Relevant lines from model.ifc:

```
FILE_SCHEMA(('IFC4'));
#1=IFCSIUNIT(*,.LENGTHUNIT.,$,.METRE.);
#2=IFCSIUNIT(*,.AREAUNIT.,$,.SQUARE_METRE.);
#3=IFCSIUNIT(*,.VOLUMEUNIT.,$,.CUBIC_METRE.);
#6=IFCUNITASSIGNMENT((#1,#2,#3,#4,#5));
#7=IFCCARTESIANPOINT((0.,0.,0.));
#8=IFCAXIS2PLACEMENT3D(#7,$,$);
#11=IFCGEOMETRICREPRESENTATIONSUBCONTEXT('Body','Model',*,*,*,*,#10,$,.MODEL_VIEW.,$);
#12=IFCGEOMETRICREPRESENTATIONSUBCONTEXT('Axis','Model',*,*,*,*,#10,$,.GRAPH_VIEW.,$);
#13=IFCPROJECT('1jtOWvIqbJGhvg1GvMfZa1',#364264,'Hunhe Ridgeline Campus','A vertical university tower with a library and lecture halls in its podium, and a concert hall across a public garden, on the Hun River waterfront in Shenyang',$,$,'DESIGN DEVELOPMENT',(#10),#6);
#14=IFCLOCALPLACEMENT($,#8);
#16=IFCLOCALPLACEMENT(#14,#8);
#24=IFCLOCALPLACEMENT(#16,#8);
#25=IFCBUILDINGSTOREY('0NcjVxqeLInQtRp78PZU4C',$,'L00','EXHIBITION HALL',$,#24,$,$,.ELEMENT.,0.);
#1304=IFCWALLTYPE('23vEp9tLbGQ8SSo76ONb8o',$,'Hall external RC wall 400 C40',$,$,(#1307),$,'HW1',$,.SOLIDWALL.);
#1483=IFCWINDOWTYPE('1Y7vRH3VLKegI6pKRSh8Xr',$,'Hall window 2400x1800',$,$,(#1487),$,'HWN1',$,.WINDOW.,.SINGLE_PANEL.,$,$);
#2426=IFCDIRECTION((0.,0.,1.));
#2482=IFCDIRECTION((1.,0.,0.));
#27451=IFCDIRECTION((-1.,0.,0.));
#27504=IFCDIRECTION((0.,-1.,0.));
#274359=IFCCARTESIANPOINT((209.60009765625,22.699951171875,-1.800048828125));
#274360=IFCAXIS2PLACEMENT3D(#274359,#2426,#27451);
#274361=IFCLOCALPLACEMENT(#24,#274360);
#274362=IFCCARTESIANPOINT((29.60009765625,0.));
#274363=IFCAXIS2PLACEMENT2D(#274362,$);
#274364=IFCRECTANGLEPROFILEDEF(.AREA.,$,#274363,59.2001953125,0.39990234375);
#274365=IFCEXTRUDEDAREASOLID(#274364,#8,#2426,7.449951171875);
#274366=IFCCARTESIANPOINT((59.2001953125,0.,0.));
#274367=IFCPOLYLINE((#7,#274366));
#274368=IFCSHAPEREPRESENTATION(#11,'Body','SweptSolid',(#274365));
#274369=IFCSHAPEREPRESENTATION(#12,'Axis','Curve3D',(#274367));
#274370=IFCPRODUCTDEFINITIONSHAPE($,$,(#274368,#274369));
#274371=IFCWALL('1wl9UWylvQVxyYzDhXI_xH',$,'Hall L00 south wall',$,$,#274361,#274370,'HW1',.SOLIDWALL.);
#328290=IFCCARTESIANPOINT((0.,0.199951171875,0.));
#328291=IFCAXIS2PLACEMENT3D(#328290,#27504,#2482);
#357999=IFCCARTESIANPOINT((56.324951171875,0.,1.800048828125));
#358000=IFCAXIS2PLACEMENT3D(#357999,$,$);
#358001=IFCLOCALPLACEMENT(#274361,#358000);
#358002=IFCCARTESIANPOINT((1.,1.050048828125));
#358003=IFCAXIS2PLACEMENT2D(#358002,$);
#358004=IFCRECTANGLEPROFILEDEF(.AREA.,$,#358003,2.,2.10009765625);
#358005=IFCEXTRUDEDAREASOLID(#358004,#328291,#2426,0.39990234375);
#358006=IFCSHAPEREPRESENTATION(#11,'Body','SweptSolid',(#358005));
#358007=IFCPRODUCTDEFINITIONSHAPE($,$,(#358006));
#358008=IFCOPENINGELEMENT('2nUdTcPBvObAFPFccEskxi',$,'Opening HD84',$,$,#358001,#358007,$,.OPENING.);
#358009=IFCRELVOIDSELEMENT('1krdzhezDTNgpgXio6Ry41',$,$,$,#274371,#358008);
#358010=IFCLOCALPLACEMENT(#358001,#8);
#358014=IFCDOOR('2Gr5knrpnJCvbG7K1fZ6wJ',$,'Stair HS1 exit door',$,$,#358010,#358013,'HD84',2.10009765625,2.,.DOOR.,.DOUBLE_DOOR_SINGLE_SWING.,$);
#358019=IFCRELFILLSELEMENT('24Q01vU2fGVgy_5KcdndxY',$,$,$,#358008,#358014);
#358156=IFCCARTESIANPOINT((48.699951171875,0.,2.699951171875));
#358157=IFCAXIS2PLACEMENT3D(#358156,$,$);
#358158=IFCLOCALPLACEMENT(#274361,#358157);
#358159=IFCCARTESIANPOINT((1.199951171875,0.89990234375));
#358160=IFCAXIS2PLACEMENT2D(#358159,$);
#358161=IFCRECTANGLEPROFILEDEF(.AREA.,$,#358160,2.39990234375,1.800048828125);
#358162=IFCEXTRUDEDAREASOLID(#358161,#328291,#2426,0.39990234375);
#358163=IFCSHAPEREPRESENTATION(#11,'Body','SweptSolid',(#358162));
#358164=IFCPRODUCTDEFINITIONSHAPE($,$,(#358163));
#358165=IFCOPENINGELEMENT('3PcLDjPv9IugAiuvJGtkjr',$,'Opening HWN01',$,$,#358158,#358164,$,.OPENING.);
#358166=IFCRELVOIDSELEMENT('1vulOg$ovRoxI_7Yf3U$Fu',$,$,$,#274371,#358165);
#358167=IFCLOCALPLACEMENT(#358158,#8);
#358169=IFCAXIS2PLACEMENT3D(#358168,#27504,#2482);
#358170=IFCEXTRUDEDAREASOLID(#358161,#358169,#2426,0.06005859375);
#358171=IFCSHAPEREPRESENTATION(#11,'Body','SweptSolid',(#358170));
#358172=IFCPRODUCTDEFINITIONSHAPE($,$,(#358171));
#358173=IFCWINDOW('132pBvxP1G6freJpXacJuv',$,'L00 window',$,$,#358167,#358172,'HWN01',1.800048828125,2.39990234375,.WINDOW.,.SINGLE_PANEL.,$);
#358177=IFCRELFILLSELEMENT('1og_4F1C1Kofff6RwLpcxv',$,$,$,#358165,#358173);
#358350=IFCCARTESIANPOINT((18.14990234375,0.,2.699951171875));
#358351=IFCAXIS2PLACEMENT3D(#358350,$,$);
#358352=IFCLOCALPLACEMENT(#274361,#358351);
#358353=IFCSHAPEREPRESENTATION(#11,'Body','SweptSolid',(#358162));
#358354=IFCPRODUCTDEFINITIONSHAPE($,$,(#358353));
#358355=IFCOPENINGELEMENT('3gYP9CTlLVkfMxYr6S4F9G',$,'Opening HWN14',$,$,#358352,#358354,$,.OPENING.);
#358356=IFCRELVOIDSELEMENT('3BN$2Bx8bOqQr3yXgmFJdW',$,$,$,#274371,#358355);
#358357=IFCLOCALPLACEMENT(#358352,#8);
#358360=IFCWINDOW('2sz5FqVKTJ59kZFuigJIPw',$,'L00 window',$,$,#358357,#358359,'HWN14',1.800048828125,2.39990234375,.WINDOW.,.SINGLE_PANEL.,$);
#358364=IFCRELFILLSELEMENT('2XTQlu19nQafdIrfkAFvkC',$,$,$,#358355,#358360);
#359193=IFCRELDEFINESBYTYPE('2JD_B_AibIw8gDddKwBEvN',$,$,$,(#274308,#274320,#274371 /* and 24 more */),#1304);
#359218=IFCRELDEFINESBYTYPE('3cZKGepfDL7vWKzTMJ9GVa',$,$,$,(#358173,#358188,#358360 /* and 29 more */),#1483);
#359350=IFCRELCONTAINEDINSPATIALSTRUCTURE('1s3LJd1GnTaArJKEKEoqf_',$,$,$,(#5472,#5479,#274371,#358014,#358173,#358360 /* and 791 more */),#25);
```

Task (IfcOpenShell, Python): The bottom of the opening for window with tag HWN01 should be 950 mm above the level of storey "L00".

```python
import numpy as np
import ifcopenshell
import ifcopenshell.api.geometry
import ifcopenshell.geom
import ifcopenshell.util.element
import ifcopenshell.util.placement
import ifcopenshell.util.shape
import ifcopenshell.util.unit

model = ifcopenshell.open("model.ifc")
unit_scale = ifcopenshell.util.unit.calculate_unit_scale(model)

window = model.by_guid("132pBvxP1G6freJpXacJuv")
opening = window.FillsVoids[0].RelatingOpeningElement
storey = ifcopenshell.util.element.get_container(window, ifc_class="IfcBuildingStorey")
level = ifcopenshell.util.placement.get_local_placement(storey.ObjectPlacement)[2, 3]

# The opening's origin need not be at the sill, so measure its lowest point.
shape = ifcopenshell.geom.create_shape(ifcopenshell.geom.settings(), opening)
bottom = ifcopenshell.util.shape.get_shape_bottom_elevation(shape, shape.geometry) / unit_scale
dz = level + 0.95 / unit_scale - bottom

shift = np.array([0.0, 0.0, dz])
# The window is placed relative to its opening, so it follows when the opening moves.
matrix = ifcopenshell.util.placement.get_local_placement(opening.ObjectPlacement)
matrix[:3, 3] += shift
ifcopenshell.api.geometry.edit_object_placement(
    model, product=opening, matrix=matrix, is_si=False, should_transform_children=True
)

print(f"moved by {dz * unit_scale:+.3f} m")

model.write("model_rev.ifc")
```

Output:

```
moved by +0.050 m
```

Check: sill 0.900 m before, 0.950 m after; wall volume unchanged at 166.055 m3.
